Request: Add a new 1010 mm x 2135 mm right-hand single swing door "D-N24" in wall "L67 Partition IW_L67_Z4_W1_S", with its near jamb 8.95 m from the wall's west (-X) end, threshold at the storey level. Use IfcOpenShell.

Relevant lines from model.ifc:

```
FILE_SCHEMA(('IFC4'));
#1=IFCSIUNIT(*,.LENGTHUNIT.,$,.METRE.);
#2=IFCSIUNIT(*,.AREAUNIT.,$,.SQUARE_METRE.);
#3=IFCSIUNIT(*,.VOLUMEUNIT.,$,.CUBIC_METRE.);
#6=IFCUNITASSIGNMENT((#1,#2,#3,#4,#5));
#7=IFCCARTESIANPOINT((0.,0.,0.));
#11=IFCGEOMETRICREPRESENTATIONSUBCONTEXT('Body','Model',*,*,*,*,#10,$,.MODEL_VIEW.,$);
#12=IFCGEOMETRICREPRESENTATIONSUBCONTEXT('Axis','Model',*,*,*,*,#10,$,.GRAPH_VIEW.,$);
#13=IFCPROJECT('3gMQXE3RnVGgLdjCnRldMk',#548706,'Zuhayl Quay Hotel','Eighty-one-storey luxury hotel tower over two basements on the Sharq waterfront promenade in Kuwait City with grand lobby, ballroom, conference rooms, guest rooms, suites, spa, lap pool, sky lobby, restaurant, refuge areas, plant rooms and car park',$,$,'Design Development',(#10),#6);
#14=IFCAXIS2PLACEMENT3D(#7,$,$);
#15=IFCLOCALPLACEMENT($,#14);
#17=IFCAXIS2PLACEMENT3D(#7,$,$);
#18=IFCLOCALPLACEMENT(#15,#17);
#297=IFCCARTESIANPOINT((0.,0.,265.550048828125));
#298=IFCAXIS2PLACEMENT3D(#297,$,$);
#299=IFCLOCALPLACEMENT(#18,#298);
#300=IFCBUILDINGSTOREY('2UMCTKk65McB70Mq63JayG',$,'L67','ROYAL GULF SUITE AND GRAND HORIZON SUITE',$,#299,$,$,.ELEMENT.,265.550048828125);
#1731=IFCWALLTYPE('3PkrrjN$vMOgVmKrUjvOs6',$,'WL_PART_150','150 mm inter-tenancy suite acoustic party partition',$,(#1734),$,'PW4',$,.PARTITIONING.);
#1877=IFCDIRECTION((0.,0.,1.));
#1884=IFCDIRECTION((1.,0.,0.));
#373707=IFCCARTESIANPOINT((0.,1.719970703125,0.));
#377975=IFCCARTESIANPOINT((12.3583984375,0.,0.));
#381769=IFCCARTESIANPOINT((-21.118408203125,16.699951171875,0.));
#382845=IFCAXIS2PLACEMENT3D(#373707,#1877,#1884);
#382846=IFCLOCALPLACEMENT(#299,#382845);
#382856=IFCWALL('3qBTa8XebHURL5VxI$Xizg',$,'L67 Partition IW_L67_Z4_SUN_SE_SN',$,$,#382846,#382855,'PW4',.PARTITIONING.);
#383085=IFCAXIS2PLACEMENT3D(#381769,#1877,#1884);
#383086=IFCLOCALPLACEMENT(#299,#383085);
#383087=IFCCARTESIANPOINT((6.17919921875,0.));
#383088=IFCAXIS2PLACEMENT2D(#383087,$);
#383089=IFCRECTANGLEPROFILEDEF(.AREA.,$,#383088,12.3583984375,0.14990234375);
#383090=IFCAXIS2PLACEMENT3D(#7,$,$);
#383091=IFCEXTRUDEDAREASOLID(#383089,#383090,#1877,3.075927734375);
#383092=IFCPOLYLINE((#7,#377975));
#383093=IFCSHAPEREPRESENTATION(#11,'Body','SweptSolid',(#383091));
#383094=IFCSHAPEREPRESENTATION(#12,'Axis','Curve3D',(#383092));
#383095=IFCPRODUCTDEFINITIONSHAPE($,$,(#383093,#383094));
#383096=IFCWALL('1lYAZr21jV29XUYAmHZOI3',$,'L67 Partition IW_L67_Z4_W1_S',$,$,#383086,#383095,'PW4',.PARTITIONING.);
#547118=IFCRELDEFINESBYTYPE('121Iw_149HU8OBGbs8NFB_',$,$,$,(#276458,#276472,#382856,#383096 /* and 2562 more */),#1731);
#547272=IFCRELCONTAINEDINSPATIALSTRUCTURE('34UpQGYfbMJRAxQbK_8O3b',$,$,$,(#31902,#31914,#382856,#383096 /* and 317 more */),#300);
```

```python
import numpy as np
import ifcopenshell
import ifcopenshell.api.feature
import ifcopenshell.api.geometry
import ifcopenshell.api.root
import ifcopenshell.api.spatial
import ifcopenshell.geom
import ifcopenshell.util.element
import ifcopenshell.util.placement
import ifcopenshell.util.representation
import ifcopenshell.util.shape
import ifcopenshell.util.unit

model = ifcopenshell.open("model.ifc")
unit_scale = ifcopenshell.util.unit.calculate_unit_scale(model)
settings = ifcopenshell.geom.settings()


def volume(element):
    """Net volume in cubic metres, openings subtracted."""
    shape = ifcopenshell.geom.create_shape(settings, element)
    return ifcopenshell.util.shape.get_volume(shape.geometry)


wall = model.by_guid("1lYAZr21jV29XUYAmHZOI3")
storey = ifcopenshell.util.element.get_container(wall, ifc_class="IfcBuildingStorey")
context = ifcopenshell.util.representation.get_context(model, "Model", "Body", "MODEL_VIEW")
before = volume(wall)

width, height, from_end, sill = 1.01, 2.135, 8.95, 0.0  # metres

# The wall runs along its own X axis, and the end named is its -X end.
wall_shape = ifcopenshell.geom.create_shape(settings, wall)
x, y, z = ifcopenshell.util.shape.get_vertices(wall_shape.geometry).T
start = x.min() + from_end
face, thickness = float(y.min()), float(y.max() - y.min())
wall_matrix = ifcopenshell.util.placement.get_local_placement(wall.ObjectPlacement)
level = ifcopenshell.util.placement.get_local_placement(storey.ObjectPlacement)[2, 3]


def in_wall(x, y):
    """Placement at x, y metres in the wall's axes, at sill height."""
    matrix = wall_matrix.copy()
    matrix[:, 3] = wall_matrix @ np.array([x / unit_scale, y / unit_scale, 0.0, 1.0])
    matrix[2, 3] = level + sill / unit_scale
    return matrix


# Opening: a box that overshoots both wall faces by 50 mm.
opening = ifcopenshell.api.root.create_entity(model, ifc_class="IfcOpeningElement", predefined_type="OPENING")
box = ifcopenshell.api.geometry.add_wall_representation(
    model, context=context, length=width, height=height, thickness=thickness + 0.1
)
ifcopenshell.api.geometry.assign_representation(model, product=opening, representation=box)
ifcopenshell.api.geometry.edit_object_placement(model, product=opening, matrix=in_wall(start, face - 0.05), is_si=False)
ifcopenshell.api.feature.add_feature(model, feature=opening, element=wall)

door = ifcopenshell.api.root.create_entity(model, ifc_class="IfcDoor", name="D-N24", predefined_type="DOOR")
door.OverallWidth, door.OverallHeight = width / unit_scale, height / unit_scale
door.OperationType = "SINGLE_SWING_RIGHT"
body = ifcopenshell.api.geometry.add_door_representation(
    model,
    context=context,
    overall_width=door.OverallWidth,
    overall_height=door.OverallHeight,
    operation_type="SINGLE_SWING_RIGHT",
    lining_properties={"LiningDepth": thickness / unit_scale, "ThresholdDepth": thickness / unit_scale},
)
ifcopenshell.api.geometry.assign_representation(model, product=door, representation=body)
ifcopenshell.api.spatial.assign_container(model, products=[door], relating_structure=storey)
ifcopenshell.api.feature.add_filling(model, opening=opening, element=door)

# The lining spans the wall, so the door starts at the wall face.
ifcopenshell.api.geometry.edit_object_placement(model, product=door, matrix=in_wall(start, face), is_si=False)

after = volume(wall)

print(f"wall volume {before:.3f} -> {after:.3f} m3")

model.write("model_updated.ifc")
```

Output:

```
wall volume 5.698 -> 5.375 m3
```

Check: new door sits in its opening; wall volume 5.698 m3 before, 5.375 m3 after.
